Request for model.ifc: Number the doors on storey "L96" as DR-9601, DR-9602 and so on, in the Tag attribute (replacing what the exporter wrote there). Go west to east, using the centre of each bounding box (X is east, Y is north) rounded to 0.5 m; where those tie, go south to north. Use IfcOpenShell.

First a look at what the model holds.

```python
import ifcopenshell
import ifcopenshell.util.element
import ifcopenshell.util.placement

model = ifcopenshell.open("model.ifc")
print(model.schema)
storey = next(s for s in model.by_type("IfcBuildingStorey") if s.Name == "L96")
doors = [e for e in ifcopenshell.util.element.get_decomposition(storey) if e.is_a("IfcDoor")]
for e in sorted(doors, key=lambda e: e.id()):
    origin = ifcopenshell.util.placement.get_local_placement(e.ObjectPlacement)[:3, 3]
    print(e.id(), e.Tag, e.Name, origin.round(2) + 0.0, sep=" | ")
```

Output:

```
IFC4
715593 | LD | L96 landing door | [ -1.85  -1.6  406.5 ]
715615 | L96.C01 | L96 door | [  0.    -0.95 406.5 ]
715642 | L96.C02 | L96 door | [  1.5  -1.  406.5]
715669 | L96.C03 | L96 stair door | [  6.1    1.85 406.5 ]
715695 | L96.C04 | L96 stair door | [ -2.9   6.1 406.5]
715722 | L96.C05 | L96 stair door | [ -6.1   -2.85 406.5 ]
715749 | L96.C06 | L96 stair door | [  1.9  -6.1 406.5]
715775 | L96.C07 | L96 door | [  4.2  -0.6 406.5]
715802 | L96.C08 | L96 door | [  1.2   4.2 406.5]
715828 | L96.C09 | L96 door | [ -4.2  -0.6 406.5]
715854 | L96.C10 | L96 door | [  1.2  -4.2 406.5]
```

```python
import ifcopenshell
import ifcopenshell.geom
import ifcopenshell.util.element
import ifcopenshell.util.shape

model = ifcopenshell.open("model.ifc")
settings = ifcopenshell.geom.settings()
settings.set("use-world-coords", True)


def centre(element):
    shape = ifcopenshell.geom.create_shape(settings, element)
    return ifcopenshell.util.shape.get_bbox_centroid(shape.geometry)


storey = next(s for s in model.by_type("IfcBuildingStorey") if s.Name == "L96")
doors = [e for e in ifcopenshell.util.element.get_decomposition(storey) if e.is_a("IfcDoor")]

# Insertion points can sit at a corner or the storey origin, so sort by the geometry (in metres).
centres = {e: centre(e) for e in doors}
doors.sort(key=lambda e: (round(centres[e][0] / 0.5), centres[e][1]))

for i, e in enumerate(doors, start=1):
    number = f"DR-96{i:02d}"
    e.Tag = number
    print(e.id(), number)

model.write("model_v2.ifc")
```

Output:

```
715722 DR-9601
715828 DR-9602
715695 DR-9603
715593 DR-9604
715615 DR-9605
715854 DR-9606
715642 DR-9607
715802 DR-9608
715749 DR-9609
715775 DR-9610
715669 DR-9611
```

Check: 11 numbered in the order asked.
